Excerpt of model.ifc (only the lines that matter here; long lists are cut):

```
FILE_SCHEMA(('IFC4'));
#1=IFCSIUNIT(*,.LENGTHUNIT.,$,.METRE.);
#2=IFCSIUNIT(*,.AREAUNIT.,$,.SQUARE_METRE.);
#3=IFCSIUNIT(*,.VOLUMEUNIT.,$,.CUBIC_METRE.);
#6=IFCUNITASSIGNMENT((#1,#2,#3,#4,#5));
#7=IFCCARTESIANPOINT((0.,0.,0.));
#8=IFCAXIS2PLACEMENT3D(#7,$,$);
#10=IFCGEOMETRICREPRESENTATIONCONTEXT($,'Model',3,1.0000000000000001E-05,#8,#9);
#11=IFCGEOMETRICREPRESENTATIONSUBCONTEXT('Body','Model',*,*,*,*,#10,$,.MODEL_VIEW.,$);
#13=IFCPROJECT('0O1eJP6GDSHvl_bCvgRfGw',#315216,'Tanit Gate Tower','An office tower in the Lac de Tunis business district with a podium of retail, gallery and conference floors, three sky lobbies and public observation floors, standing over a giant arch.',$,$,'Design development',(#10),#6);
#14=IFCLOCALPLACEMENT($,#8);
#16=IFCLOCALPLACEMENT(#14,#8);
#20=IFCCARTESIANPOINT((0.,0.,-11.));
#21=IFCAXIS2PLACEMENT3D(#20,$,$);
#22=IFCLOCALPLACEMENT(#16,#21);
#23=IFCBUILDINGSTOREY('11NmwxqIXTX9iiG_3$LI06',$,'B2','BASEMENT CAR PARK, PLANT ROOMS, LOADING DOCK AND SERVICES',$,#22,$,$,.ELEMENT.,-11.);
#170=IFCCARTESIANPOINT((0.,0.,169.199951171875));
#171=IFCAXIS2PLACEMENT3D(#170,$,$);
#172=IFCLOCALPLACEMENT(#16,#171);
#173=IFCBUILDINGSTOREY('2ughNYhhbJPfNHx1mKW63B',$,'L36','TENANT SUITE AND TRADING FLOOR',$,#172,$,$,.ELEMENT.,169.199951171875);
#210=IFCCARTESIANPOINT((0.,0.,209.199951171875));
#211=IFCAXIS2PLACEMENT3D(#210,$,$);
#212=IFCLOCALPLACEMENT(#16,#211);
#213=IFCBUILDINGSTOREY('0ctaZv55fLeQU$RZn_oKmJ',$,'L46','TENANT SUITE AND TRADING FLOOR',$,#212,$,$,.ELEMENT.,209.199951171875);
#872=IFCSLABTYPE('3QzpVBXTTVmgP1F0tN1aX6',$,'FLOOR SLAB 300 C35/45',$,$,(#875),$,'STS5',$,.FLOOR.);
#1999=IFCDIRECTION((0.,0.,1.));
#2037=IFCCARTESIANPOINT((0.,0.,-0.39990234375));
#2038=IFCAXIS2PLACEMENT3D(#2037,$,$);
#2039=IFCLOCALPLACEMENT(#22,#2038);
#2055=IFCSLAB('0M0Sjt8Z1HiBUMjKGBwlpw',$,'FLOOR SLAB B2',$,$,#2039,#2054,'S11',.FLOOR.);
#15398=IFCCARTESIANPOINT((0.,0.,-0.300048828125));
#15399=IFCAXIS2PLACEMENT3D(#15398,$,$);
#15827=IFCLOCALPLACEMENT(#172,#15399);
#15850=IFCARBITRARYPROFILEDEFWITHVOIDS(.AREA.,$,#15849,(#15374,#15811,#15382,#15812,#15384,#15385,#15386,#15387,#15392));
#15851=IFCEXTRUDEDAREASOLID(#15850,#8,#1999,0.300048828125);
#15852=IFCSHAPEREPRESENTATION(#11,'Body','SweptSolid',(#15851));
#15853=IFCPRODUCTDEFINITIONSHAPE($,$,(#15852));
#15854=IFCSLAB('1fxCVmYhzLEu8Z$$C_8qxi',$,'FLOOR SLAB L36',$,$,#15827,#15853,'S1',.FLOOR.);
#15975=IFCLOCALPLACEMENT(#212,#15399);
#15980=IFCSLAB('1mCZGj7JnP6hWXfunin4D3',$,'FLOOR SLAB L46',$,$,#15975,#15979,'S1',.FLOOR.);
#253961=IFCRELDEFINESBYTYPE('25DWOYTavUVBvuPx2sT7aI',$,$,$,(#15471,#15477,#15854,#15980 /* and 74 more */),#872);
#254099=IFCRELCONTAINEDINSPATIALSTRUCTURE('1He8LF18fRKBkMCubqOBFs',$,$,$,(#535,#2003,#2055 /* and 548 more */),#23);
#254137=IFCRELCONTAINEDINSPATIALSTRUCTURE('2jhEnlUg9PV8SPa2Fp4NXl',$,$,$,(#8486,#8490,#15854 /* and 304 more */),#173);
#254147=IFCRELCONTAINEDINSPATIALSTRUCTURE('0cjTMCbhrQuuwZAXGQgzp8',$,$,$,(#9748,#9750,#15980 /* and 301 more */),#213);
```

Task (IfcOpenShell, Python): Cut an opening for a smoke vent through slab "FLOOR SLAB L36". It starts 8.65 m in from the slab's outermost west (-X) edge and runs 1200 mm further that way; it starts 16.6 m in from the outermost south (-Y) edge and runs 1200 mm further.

```python
import numpy as np
import ifcopenshell
import ifcopenshell.api.feature
import ifcopenshell.api.geometry
import ifcopenshell.api.root
import ifcopenshell.geom
import ifcopenshell.util.placement
import ifcopenshell.util.representation
import ifcopenshell.util.shape
import ifcopenshell.util.unit

model = ifcopenshell.open("model.ifc")
unit_scale = ifcopenshell.util.unit.calculate_unit_scale(model)
settings = ifcopenshell.geom.settings()


def volume(element):
    """Net volume in cubic metres, openings subtracted."""
    shape = ifcopenshell.geom.create_shape(settings, element)
    return ifcopenshell.util.shape.get_volume(shape.geometry)


slab = model.by_id(15854)
before = volume(slab)

# Extent in the slab's own axes, in metres. The edges named are its -X and -Y sides.
slab_shape = ifcopenshell.geom.create_shape(settings, slab)
vertices = ifcopenshell.util.shape.get_vertices(slab_shape.geometry)
x_min, y_min, bottom = vertices.min(axis=0)
top = vertices[:, 2].max()

opening = ifcopenshell.api.root.create_entity(model, ifc_class="IfcOpeningElement", name="Smoke vent opening", predefined_type="OPENING")
context = ifcopenshell.util.representation.get_context(model, "Model", "Body", "MODEL_VIEW")
width, depth = 1.2, 1.2
outline = [(0.0, 0.0), (width, 0.0), (width, depth), (0.0, depth), (0.0, 0.0)]
# Overshoot both faces by 50 mm so the cut is clean.
shape = ifcopenshell.api.geometry.add_slab_representation(
    model, context=context, depth=top - bottom + 0.1, polyline=outline
)
ifcopenshell.api.geometry.assign_representation(model, product=opening, representation=shape)

matrix = ifcopenshell.util.placement.get_local_placement(slab.ObjectPlacement)
matrix[:, 3] = matrix @ np.append(np.array([x_min + 8.65, y_min + 16.6, bottom - 0.05]) / unit_scale, 1.0)
ifcopenshell.api.geometry.edit_object_placement(model, product=opening, matrix=matrix, is_si=False)
ifcopenshell.api.feature.add_feature(model, feature=opening, element=slab)

after = volume(slab)

print(f"slab volume {before:.3f} -> {after:.3f} m3")

model.write("model_edited.ifc")
```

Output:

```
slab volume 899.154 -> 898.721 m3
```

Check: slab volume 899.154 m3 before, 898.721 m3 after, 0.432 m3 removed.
